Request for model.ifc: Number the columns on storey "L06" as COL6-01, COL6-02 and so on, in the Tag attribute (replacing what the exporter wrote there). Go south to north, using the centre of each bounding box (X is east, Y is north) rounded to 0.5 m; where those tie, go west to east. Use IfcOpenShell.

First a look at what the model holds.

```python
import ifcopenshell
import ifcopenshell.util.element
import ifcopenshell.util.placement

model = ifcopenshell.open("model.ifc")
print(model.schema)
storey = next(s for s in model.by_type("IfcBuildingStorey") if s.Name == "L06")
columns = [e for e in ifcopenshell.util.element.get_decomposition(storey) if e.is_a("IfcColumn")]
for e in sorted(columns, key=lambda e: e.id()):
    origin = ifcopenshell.util.placement.get_local_placement(e.ObjectPlacement)[:3, 3]
    print(e.id(), e.Tag, e.Name, origin.round(2) + 0.0, sep=" | ")
```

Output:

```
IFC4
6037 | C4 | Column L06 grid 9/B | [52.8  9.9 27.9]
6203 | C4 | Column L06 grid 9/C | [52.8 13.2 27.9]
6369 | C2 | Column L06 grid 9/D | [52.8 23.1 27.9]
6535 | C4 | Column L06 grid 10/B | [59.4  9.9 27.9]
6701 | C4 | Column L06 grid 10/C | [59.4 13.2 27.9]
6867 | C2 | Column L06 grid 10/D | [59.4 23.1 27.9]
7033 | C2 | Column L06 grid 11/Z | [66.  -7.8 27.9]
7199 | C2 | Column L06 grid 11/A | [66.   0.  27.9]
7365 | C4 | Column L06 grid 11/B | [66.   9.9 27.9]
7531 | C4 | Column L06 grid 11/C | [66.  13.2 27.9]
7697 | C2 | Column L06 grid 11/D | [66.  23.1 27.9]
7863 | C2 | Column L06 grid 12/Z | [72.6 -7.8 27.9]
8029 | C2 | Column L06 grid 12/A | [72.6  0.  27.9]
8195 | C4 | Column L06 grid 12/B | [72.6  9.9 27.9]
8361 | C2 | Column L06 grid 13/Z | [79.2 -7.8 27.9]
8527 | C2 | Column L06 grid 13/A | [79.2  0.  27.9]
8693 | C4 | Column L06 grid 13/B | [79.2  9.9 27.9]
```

```python
import ifcopenshell
import ifcopenshell.geom
import ifcopenshell.util.element
import ifcopenshell.util.shape

model = ifcopenshell.open("model.ifc")
settings = ifcopenshell.geom.settings()
settings.set("use-world-coords", True)


def centre(element):
    shape = ifcopenshell.geom.create_shape(settings, element)
    return ifcopenshell.util.shape.get_bbox_centroid(shape.geometry)


storey = next(s for s in model.by_type("IfcBuildingStorey") if s.Name == "L06")
columns = [e for e in ifcopenshell.util.element.get_decomposition(storey) if e.is_a("IfcColumn")]

# Insertion points can sit at a corner or the storey origin, so sort by the geometry (in metres).
centres = {e: centre(e) for e in columns}
columns.sort(key=lambda e: (round(centres[e][1] / 0.5), centres[e][0]))

for i, e in enumerate(columns, start=1):
    number = f"COL6-{i:02d}"
    e.Tag = number
    print(e.id(), number)

model.write("model-out.ifc")
```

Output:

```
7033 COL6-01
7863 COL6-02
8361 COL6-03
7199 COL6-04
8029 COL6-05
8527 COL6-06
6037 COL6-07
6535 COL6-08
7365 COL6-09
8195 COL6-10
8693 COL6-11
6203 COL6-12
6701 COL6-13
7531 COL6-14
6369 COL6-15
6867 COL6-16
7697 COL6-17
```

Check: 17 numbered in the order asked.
